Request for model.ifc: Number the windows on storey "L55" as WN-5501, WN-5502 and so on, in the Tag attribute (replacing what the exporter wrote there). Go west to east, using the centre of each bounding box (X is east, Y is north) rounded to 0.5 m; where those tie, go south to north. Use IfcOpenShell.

First a look at what the model holds.

```python
import ifcopenshell
import ifcopenshell.util.element
import ifcopenshell.util.placement

model = ifcopenshell.open("model.ifc")
print(model.schema)
storey = next(s for s in model.by_type("IfcBuildingStorey") if s.Name == "L55")
windows = [e for e in ifcopenshell.util.element.get_decomposition(storey) if e.is_a("IfcWindow")]
for e in sorted(windows, key=lambda e: e.id()):
    origin = ifcopenshell.util.placement.get_local_placement(e.ObjectPlacement)[:3, 3]
    print(e.id(), e.Tag, e.Name, origin.round(2) + 0.0, sep=" | ")
```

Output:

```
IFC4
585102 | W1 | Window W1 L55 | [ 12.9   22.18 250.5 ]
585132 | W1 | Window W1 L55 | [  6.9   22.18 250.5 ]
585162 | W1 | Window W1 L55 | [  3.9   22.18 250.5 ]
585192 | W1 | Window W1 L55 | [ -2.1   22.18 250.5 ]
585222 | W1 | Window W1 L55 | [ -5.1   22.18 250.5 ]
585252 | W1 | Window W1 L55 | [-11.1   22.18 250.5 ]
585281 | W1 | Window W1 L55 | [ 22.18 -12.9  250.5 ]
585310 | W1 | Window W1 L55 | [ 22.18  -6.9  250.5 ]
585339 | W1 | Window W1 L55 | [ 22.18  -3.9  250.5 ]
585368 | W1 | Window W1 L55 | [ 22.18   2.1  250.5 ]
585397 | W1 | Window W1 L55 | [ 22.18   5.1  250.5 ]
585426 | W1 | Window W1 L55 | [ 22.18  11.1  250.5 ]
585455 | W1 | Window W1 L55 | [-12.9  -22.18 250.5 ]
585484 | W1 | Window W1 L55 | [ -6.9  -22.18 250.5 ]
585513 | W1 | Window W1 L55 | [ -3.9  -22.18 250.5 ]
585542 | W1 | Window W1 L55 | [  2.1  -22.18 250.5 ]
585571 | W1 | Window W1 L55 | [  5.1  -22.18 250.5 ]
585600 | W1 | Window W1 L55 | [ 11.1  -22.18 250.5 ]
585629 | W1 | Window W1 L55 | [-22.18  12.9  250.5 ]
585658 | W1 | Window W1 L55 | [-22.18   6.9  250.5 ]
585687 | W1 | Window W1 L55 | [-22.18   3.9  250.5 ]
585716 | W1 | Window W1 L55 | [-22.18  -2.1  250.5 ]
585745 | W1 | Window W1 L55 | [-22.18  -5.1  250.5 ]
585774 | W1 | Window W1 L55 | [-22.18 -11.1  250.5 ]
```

```python
import ifcopenshell
import ifcopenshell.geom
import ifcopenshell.util.element
import ifcopenshell.util.shape

model = ifcopenshell.open("model.ifc")
settings = ifcopenshell.geom.settings()
settings.set("use-world-coords", True)


def centre(element):
    shape = ifcopenshell.geom.create_shape(settings, element)
    return ifcopenshell.util.shape.get_bbox_centroid(shape.geometry)


storey = next(s for s in model.by_type("IfcBuildingStorey") if s.Name == "L55")
windows = [e for e in ifcopenshell.util.element.get_decomposition(storey) if e.is_a("IfcWindow")]

# Insertion points can sit at a corner or the storey origin, so sort by the geometry (in metres).
centres = {e: centre(e) for e in windows}
windows.sort(key=lambda e: (round(centres[e][0] / 0.5), centres[e][1]))

for i, e in enumerate(windows, start=1):
    number = f"WN-55{i:02d}"
    e.Tag = number
    print(e.id(), number)

model.write("model_edited.ifc")
```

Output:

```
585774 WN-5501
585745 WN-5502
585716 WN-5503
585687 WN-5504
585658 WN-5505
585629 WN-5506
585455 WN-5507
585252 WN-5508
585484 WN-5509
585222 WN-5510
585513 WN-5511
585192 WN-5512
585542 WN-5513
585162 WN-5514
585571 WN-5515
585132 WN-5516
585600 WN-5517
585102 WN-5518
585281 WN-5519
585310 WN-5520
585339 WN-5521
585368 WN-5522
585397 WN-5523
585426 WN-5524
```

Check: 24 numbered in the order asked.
